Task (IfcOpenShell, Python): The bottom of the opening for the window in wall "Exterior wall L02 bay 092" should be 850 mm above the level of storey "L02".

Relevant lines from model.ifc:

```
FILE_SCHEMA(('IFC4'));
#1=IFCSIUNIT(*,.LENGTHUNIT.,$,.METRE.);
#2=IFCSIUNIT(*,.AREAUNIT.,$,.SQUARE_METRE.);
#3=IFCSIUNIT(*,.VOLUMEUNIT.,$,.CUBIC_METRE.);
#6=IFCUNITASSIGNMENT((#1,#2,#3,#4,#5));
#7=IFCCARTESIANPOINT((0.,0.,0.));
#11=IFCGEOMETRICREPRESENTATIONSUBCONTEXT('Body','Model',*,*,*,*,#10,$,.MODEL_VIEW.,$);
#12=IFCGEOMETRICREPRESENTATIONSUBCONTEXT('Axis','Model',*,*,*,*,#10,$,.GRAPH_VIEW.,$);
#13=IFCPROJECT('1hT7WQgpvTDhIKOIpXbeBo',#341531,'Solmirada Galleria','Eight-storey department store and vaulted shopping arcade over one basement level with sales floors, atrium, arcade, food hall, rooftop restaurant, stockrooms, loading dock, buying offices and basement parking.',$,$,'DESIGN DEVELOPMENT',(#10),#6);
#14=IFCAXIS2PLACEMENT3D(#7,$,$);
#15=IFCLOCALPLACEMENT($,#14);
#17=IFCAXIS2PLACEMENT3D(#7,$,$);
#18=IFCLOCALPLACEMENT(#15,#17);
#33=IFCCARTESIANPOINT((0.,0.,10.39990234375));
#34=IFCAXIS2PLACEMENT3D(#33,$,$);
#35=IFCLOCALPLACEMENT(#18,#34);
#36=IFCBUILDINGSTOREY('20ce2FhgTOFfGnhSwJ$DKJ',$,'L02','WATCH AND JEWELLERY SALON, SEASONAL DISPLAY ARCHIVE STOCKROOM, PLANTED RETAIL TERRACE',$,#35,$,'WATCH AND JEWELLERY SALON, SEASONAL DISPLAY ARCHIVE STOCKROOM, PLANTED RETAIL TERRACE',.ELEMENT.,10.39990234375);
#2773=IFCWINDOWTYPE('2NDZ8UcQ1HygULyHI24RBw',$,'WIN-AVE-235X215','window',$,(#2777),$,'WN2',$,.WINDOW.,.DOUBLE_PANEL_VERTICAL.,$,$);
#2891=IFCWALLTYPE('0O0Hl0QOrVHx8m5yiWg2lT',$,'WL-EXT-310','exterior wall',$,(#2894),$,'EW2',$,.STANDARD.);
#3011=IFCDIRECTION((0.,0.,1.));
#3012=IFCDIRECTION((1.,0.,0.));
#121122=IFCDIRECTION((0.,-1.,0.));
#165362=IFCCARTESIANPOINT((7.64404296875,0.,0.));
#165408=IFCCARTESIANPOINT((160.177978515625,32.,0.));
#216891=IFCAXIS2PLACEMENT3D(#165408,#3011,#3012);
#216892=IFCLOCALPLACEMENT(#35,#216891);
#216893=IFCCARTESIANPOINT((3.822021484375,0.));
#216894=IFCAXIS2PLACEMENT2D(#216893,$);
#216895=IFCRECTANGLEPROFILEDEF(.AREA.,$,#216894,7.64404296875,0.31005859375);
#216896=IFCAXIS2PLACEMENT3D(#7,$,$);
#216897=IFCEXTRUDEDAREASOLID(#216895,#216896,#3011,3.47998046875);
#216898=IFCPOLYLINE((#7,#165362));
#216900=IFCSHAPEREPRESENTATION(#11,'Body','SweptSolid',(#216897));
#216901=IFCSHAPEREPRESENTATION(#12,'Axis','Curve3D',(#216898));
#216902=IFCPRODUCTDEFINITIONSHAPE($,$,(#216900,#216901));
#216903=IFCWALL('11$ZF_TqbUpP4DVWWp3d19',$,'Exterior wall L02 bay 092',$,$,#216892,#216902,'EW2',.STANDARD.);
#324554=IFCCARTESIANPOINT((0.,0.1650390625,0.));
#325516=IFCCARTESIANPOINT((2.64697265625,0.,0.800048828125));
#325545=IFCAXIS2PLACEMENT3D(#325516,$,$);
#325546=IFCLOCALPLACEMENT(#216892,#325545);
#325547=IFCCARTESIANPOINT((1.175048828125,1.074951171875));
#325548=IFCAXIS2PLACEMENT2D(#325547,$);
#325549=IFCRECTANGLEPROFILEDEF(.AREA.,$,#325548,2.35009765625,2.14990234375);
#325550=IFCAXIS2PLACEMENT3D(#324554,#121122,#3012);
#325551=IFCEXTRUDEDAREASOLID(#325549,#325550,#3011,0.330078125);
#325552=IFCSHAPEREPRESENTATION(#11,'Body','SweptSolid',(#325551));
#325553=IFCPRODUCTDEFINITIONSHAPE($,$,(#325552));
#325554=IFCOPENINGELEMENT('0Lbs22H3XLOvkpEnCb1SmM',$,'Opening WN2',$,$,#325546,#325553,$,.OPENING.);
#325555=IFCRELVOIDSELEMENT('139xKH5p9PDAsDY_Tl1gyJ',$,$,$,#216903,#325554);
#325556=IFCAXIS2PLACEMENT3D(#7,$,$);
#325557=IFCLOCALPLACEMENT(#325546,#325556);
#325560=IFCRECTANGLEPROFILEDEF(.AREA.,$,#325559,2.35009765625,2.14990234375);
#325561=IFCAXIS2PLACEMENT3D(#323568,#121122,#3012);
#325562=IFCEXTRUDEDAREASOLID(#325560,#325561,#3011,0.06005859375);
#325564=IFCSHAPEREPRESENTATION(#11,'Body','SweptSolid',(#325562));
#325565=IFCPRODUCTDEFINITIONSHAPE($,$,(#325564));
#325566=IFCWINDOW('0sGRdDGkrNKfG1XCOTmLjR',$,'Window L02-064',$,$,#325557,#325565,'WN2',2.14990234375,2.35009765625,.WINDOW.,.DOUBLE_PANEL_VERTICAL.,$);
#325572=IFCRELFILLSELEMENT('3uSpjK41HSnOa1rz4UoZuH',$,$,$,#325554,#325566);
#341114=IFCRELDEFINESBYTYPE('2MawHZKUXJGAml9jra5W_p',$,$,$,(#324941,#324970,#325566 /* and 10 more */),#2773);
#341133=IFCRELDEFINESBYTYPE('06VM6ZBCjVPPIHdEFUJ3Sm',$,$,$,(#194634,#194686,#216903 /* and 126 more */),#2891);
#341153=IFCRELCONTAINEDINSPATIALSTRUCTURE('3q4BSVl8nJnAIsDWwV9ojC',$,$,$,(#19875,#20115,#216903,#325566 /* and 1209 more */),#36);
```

```python
import numpy as np
import ifcopenshell
import ifcopenshell.api.geometry
import ifcopenshell.geom
import ifcopenshell.util.element
import ifcopenshell.util.placement
import ifcopenshell.util.shape
import ifcopenshell.util.unit

model = ifcopenshell.open("model.ifc")
unit_scale = ifcopenshell.util.unit.calculate_unit_scale(model)

window = model.by_guid("0sGRdDGkrNKfG1XCOTmLjR")
opening = window.FillsVoids[0].RelatingOpeningElement
storey = ifcopenshell.util.element.get_container(window, ifc_class="IfcBuildingStorey")
level = ifcopenshell.util.placement.get_local_placement(storey.ObjectPlacement)[2, 3]

# The opening's origin need not be at the sill, so measure its lowest point.
shape = ifcopenshell.geom.create_shape(ifcopenshell.geom.settings(), opening)
bottom = ifcopenshell.util.shape.get_shape_bottom_elevation(shape, shape.geometry) / unit_scale
dz = level + 0.85 - bottom

shift = np.array([0.0, 0.0, dz])
# The window is placed relative to its opening, so it follows when the opening moves.
matrix = ifcopenshell.util.placement.get_local_placement(opening.ObjectPlacement)
matrix[:3, 3] += shift
ifcopenshell.api.geometry.edit_object_placement(
    model, product=opening, matrix=matrix, is_si=False, should_transform_children=True
)

print(f"moved by {dz * unit_scale:+.3f} m")

model.write("model_updated.ifc")
```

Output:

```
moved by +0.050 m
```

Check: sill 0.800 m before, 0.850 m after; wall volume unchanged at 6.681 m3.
